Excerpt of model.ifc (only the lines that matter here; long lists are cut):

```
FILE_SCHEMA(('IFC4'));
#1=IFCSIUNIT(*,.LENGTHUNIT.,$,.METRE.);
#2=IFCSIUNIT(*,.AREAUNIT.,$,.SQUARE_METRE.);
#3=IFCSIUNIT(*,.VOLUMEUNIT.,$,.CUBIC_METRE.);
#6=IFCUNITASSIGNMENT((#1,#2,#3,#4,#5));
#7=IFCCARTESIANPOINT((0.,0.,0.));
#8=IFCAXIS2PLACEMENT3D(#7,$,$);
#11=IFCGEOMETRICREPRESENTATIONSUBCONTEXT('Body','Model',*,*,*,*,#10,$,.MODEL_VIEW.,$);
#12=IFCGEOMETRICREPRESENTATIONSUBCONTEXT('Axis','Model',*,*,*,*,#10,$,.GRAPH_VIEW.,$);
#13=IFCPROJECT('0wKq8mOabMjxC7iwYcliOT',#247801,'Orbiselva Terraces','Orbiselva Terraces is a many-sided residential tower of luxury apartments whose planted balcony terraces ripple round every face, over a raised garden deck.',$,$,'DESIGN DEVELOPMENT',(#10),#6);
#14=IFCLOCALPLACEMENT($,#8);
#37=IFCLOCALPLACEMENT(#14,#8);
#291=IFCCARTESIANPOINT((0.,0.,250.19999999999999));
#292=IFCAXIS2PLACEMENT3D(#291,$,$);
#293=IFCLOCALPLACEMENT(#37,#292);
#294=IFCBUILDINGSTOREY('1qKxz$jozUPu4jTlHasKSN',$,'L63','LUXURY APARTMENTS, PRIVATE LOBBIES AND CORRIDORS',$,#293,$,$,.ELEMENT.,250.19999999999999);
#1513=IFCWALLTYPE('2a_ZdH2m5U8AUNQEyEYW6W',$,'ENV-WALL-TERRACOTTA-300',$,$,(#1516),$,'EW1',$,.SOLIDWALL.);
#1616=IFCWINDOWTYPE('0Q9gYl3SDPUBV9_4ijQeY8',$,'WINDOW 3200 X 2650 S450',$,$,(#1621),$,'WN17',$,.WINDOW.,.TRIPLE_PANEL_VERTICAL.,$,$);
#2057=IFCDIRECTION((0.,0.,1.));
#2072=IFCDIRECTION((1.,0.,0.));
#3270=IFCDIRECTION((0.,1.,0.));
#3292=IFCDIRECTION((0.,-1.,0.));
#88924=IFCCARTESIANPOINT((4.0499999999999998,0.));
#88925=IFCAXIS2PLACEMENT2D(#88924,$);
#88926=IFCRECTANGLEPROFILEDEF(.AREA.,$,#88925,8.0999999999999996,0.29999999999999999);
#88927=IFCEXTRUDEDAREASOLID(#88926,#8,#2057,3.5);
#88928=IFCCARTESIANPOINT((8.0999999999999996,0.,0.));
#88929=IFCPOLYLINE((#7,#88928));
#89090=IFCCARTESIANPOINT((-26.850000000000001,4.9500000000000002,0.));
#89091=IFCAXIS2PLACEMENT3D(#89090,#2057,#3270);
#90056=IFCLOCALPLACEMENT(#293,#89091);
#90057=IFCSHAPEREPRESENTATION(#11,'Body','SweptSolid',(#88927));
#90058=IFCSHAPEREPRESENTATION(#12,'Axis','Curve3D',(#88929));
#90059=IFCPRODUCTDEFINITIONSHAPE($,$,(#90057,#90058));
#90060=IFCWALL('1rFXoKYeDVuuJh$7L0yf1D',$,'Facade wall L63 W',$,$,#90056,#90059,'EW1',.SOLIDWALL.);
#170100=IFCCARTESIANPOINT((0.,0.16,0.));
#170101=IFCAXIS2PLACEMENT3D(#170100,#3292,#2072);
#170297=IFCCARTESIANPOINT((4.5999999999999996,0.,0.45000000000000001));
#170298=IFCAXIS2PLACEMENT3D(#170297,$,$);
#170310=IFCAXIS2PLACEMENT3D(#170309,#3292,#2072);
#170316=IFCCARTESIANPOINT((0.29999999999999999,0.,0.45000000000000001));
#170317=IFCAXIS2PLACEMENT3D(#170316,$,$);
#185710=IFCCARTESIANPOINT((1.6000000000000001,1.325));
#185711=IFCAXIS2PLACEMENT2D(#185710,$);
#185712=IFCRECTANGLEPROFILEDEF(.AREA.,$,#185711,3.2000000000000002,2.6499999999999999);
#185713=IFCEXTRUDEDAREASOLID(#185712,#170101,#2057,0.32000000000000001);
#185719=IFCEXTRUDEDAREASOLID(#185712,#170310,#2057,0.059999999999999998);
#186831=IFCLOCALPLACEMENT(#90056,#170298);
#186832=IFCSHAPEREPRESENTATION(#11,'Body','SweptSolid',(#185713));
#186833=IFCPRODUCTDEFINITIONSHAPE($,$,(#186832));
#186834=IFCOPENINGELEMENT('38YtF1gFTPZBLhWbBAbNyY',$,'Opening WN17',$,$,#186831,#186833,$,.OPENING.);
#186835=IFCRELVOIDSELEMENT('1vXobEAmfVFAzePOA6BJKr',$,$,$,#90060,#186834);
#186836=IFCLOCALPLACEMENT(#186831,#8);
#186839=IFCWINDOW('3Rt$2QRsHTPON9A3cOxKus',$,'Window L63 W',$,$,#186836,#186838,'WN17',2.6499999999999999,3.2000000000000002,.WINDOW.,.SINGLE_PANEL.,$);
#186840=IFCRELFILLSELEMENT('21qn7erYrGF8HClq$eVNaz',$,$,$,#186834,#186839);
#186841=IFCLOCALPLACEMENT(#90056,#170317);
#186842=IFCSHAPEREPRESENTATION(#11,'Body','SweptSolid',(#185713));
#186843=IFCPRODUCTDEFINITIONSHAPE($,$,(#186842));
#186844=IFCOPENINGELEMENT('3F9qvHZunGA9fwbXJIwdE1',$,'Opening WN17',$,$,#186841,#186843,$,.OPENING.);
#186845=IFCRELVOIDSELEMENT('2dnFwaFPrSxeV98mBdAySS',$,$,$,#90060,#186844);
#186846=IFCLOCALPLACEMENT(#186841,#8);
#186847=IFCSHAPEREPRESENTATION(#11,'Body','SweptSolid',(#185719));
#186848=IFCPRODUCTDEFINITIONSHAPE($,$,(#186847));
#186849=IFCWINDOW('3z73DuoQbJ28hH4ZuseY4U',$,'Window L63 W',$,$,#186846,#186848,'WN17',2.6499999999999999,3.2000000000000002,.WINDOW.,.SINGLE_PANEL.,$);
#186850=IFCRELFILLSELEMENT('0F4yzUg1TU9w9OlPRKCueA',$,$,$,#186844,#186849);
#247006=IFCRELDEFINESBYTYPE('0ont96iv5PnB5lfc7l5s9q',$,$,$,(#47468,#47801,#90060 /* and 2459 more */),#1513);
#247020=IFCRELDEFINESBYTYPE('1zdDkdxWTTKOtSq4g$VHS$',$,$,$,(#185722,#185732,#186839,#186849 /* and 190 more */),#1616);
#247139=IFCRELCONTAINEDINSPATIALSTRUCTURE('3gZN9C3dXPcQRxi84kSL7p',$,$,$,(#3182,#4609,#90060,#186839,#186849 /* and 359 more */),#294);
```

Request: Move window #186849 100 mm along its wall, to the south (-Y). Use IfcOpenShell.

```python
import ifcopenshell
import ifcopenshell.api.geometry
import ifcopenshell.util.placement

model = ifcopenshell.open("model.ifc")

window = model.by_guid("3z73DuoQbJ28hH4ZuseY4U")
opening = window.FillsVoids[0].RelatingOpeningElement
wall = opening.VoidsElements[0].RelatingBuildingElement

wall_matrix = ifcopenshell.util.placement.get_local_placement(wall.ObjectPlacement)
shift = wall_matrix[:3, 0] * -0.1
before = ifcopenshell.util.placement.get_local_placement(window.ObjectPlacement)[:3, 3].copy()

# The window is placed relative to its opening, so it follows when the opening moves.
matrix = ifcopenshell.util.placement.get_local_placement(opening.ObjectPlacement)
matrix[:3, 3] += shift
ifcopenshell.api.geometry.edit_object_placement(
    model, product=opening, matrix=matrix, is_si=False, should_transform_children=True
)

after = ifcopenshell.util.placement.get_local_placement(window.ObjectPlacement)[:3, 3]
print("window moved by", (after - before).round(3) + 0.0)

model.write("model-out.ifc")
```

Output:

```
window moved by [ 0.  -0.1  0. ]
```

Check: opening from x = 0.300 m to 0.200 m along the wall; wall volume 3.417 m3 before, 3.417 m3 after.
